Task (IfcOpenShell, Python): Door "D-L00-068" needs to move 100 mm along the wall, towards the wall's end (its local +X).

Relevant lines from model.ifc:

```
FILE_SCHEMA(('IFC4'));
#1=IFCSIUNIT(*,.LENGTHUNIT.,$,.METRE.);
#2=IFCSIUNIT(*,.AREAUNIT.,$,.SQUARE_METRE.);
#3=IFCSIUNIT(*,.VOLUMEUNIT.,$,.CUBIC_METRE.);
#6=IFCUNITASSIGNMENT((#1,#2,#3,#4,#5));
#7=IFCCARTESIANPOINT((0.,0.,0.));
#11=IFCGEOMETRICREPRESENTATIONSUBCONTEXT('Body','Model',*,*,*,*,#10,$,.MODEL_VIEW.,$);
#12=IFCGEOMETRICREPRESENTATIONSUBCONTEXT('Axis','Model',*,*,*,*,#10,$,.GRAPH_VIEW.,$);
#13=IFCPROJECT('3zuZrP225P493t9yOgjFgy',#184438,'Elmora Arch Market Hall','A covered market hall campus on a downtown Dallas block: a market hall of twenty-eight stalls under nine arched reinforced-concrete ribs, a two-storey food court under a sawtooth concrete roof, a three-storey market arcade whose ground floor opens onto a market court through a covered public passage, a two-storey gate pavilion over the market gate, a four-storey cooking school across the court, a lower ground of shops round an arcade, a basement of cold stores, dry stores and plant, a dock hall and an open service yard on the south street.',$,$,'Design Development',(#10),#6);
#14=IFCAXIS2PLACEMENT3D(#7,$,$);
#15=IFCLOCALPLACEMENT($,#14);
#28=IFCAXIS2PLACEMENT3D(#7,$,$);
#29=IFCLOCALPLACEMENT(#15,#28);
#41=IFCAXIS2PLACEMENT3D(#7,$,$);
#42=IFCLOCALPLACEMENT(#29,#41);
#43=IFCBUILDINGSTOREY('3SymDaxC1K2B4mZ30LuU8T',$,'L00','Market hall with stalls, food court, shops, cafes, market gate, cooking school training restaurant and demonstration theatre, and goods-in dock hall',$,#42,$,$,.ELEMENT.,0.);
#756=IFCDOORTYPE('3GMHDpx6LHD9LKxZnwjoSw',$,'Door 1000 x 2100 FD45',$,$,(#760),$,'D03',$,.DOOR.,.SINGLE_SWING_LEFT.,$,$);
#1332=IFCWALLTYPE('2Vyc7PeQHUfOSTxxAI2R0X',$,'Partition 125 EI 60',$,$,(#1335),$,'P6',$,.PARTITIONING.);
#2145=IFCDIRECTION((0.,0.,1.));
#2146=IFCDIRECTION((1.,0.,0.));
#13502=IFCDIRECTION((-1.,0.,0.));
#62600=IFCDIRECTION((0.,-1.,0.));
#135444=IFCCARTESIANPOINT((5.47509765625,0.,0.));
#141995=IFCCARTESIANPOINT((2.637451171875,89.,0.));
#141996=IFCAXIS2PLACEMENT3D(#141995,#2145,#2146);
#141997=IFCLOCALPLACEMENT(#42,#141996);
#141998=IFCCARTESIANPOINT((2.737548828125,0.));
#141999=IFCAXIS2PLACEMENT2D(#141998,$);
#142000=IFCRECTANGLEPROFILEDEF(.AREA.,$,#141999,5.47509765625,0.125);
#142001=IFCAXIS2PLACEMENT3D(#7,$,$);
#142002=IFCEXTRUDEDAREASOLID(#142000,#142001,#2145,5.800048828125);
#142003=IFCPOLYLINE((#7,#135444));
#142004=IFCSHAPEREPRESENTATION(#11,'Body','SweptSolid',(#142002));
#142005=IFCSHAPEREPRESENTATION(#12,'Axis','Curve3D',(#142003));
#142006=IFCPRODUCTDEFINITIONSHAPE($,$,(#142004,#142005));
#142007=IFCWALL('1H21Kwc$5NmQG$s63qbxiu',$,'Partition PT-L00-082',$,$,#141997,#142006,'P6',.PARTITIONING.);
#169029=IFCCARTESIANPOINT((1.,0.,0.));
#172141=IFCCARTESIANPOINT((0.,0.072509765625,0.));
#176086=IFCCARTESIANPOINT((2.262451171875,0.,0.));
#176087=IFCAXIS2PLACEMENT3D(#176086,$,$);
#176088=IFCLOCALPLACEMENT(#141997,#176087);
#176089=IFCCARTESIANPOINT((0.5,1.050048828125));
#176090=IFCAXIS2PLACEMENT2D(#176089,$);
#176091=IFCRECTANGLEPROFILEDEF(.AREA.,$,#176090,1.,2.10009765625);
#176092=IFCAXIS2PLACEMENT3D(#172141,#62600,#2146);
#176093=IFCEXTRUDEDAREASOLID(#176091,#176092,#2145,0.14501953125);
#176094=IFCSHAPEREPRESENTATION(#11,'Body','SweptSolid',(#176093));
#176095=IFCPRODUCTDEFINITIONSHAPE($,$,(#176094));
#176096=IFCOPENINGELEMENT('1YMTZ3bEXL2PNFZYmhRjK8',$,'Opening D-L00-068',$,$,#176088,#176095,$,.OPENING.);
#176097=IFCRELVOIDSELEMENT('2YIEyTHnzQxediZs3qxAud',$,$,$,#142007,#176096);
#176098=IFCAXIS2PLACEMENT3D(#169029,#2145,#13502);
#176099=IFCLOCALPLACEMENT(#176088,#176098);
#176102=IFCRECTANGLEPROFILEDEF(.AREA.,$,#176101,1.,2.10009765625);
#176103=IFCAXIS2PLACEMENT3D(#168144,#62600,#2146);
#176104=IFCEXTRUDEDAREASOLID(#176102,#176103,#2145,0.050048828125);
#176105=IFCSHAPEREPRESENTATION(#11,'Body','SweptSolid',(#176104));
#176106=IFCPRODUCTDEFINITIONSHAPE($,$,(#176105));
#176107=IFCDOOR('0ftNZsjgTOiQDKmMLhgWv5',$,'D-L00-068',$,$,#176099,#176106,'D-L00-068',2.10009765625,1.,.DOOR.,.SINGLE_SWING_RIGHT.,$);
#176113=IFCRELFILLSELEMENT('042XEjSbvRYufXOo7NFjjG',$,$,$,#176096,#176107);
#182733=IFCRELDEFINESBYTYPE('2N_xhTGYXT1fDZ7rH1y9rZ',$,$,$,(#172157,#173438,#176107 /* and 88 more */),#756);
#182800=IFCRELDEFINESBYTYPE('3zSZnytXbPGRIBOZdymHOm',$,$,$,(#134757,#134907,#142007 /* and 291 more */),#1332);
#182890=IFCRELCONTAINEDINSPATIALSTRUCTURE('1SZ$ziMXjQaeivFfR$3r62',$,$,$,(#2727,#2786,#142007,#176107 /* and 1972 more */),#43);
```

```python
import ifcopenshell
import ifcopenshell.api.geometry
import ifcopenshell.util.placement
import ifcopenshell.util.unit

model = ifcopenshell.open("model.ifc")
unit_scale = ifcopenshell.util.unit.calculate_unit_scale(model)

door = model.by_id(176107)
opening = door.FillsVoids[0].RelatingOpeningElement
wall = opening.VoidsElements[0].RelatingBuildingElement

wall_matrix = ifcopenshell.util.placement.get_local_placement(wall.ObjectPlacement)
shift = wall_matrix[:3, 0] * 0.1 / unit_scale
before = ifcopenshell.util.placement.get_local_placement(door.ObjectPlacement)[:3, 3].copy()

# The door is placed relative to its opening, so it follows when the opening moves.
matrix = ifcopenshell.util.placement.get_local_placement(opening.ObjectPlacement)
matrix[:3, 3] += shift
ifcopenshell.api.geometry.edit_object_placement(
    model, product=opening, matrix=matrix, is_si=False, should_transform_children=True
)

after = ifcopenshell.util.placement.get_local_placement(door.ObjectPlacement)[:3, 3]
print("door moved by", (after - before).round(3) + 0.0)

model.write("model_edited.ifc")
```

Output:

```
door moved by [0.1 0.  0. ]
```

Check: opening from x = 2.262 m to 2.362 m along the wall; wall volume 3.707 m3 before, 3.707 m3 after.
